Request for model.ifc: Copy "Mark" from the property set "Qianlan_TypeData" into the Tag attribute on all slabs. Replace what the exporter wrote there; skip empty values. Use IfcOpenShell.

First a look at what the model holds.

```python
import ifcopenshell
import ifcopenshell.util.element

model = ifcopenshell.open("model.ifc")
print(model.schema)
slabs = model.by_type("IfcSlab")
print(len(slabs), "slabs")
for e in slabs[:8]:
    source = ifcopenshell.util.element.get_pset(e, "Qianlan_TypeData", "Mark")
    target = e.Tag
    print(e.id(), repr(source), repr(target), sep=" | ")
```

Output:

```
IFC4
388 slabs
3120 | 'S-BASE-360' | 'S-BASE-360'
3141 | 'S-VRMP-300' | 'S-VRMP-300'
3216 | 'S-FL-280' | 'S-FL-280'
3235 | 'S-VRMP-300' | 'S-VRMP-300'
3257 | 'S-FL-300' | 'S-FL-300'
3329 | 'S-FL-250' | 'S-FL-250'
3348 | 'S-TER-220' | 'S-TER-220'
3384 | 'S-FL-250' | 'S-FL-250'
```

```python
import ifcopenshell
import ifcopenshell.util.element

model = ifcopenshell.open("model.ifc")

count = 0
for e in model.by_type("IfcSlab"):
    value = ifcopenshell.util.element.get_pset(e, "Qianlan_TypeData", "Mark")
    current = e.Tag
    if not value or not value.strip() or current == value:
        continue
    e.Tag = value
    count += 1

print(count, "slabs updated")

model.write("model_updated.ifc")
```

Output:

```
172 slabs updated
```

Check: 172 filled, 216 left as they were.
